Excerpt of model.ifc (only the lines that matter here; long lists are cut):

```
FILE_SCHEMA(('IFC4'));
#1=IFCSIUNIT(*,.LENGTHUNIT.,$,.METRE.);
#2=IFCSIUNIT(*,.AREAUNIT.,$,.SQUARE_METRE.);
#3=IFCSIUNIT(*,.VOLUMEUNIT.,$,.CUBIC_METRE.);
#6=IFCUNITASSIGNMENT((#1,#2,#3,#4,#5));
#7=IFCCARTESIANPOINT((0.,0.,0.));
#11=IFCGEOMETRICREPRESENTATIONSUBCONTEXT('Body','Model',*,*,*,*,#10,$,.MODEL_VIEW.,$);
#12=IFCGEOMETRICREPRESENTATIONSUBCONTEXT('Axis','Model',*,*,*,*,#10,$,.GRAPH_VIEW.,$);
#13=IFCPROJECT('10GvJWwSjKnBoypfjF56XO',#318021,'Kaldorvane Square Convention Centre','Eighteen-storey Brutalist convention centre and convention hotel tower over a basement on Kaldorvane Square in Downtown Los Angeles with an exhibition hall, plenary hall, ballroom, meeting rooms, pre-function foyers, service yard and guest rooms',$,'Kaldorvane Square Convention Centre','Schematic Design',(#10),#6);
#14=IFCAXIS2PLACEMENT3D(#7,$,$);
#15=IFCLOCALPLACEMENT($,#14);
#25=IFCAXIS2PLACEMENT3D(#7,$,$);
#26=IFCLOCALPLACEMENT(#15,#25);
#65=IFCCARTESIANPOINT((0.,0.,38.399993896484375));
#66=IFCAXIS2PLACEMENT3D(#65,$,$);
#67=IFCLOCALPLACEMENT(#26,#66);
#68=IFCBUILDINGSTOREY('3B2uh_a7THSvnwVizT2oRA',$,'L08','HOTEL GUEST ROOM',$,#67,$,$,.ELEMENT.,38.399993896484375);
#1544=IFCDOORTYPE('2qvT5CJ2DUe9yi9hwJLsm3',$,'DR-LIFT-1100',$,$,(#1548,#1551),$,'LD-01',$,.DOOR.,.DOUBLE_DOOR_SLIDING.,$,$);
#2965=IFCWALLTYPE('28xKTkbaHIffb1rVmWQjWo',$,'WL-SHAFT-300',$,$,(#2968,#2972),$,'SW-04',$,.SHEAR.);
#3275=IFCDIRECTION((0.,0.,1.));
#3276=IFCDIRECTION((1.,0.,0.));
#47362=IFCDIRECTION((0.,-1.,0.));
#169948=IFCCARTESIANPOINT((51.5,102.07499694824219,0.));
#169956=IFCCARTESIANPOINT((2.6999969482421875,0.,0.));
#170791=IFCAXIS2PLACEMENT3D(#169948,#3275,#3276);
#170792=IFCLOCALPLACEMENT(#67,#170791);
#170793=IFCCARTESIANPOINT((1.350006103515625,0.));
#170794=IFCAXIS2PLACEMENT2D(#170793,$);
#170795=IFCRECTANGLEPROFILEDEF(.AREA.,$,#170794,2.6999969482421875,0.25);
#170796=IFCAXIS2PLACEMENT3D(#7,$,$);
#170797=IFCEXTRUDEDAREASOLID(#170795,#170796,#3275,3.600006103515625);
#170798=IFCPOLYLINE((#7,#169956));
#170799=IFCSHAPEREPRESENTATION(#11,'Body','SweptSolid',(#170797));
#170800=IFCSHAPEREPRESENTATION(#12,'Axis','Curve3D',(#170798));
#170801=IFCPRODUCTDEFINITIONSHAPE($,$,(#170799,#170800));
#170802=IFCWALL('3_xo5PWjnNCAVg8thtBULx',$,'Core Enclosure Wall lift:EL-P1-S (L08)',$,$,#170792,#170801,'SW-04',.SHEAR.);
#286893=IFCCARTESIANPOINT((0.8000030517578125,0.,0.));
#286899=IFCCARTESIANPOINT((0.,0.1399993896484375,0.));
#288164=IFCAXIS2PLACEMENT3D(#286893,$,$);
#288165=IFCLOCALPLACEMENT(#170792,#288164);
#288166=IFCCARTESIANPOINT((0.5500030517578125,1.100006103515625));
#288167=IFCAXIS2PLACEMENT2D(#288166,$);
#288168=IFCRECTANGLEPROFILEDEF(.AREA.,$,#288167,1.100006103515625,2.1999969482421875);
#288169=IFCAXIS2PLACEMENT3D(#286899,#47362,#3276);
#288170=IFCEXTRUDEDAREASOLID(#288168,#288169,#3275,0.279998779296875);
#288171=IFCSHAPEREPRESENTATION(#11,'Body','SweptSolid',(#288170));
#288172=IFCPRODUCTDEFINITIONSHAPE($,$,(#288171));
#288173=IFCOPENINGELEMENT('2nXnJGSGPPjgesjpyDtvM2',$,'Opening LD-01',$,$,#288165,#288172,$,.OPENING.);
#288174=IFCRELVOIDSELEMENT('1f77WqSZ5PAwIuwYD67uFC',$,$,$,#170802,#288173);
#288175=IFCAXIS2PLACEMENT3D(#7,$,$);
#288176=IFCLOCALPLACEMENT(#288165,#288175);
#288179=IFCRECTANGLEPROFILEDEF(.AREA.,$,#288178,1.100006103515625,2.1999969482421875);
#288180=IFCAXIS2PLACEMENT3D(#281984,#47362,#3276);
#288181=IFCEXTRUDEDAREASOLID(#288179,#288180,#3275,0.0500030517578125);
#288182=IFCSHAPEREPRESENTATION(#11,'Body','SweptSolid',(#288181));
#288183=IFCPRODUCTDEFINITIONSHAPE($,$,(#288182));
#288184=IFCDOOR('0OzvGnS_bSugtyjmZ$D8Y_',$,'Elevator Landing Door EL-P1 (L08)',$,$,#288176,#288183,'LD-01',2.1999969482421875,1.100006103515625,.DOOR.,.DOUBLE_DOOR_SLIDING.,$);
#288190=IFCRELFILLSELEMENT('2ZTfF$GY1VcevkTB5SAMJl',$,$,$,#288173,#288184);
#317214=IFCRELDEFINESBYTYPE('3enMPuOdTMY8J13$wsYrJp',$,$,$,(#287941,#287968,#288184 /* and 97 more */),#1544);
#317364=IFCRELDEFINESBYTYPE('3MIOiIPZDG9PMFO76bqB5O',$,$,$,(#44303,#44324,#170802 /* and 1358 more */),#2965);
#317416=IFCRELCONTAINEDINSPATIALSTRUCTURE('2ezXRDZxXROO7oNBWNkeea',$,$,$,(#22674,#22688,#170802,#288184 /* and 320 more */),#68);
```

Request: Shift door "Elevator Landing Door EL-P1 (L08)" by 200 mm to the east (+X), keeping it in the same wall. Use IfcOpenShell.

```python
import ifcopenshell
import ifcopenshell.api.geometry
import ifcopenshell.util.placement
import ifcopenshell.util.unit

model = ifcopenshell.open("model.ifc")
unit_scale = ifcopenshell.util.unit.calculate_unit_scale(model)

door = model.by_id(288184)
opening = door.FillsVoids[0].RelatingOpeningElement
wall = opening.VoidsElements[0].RelatingBuildingElement

wall_matrix = ifcopenshell.util.placement.get_local_placement(wall.ObjectPlacement)
shift = wall_matrix[:3, 0] * 0.2 / unit_scale
before = ifcopenshell.util.placement.get_local_placement(door.ObjectPlacement)[:3, 3].copy()

# The door is placed relative to its opening, so it follows when the opening moves.
matrix = ifcopenshell.util.placement.get_local_placement(opening.ObjectPlacement)
matrix[:3, 3] += shift
ifcopenshell.api.geometry.edit_object_placement(
    model, product=opening, matrix=matrix, is_si=False, should_transform_children=True
)

after = ifcopenshell.util.placement.get_local_placement(door.ObjectPlacement)[:3, 3]
print("door moved by", (after - before).round(3) + 0.0)

model.write("model-out.ifc")
```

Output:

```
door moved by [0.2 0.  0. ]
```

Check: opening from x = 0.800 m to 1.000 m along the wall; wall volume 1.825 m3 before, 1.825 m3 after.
